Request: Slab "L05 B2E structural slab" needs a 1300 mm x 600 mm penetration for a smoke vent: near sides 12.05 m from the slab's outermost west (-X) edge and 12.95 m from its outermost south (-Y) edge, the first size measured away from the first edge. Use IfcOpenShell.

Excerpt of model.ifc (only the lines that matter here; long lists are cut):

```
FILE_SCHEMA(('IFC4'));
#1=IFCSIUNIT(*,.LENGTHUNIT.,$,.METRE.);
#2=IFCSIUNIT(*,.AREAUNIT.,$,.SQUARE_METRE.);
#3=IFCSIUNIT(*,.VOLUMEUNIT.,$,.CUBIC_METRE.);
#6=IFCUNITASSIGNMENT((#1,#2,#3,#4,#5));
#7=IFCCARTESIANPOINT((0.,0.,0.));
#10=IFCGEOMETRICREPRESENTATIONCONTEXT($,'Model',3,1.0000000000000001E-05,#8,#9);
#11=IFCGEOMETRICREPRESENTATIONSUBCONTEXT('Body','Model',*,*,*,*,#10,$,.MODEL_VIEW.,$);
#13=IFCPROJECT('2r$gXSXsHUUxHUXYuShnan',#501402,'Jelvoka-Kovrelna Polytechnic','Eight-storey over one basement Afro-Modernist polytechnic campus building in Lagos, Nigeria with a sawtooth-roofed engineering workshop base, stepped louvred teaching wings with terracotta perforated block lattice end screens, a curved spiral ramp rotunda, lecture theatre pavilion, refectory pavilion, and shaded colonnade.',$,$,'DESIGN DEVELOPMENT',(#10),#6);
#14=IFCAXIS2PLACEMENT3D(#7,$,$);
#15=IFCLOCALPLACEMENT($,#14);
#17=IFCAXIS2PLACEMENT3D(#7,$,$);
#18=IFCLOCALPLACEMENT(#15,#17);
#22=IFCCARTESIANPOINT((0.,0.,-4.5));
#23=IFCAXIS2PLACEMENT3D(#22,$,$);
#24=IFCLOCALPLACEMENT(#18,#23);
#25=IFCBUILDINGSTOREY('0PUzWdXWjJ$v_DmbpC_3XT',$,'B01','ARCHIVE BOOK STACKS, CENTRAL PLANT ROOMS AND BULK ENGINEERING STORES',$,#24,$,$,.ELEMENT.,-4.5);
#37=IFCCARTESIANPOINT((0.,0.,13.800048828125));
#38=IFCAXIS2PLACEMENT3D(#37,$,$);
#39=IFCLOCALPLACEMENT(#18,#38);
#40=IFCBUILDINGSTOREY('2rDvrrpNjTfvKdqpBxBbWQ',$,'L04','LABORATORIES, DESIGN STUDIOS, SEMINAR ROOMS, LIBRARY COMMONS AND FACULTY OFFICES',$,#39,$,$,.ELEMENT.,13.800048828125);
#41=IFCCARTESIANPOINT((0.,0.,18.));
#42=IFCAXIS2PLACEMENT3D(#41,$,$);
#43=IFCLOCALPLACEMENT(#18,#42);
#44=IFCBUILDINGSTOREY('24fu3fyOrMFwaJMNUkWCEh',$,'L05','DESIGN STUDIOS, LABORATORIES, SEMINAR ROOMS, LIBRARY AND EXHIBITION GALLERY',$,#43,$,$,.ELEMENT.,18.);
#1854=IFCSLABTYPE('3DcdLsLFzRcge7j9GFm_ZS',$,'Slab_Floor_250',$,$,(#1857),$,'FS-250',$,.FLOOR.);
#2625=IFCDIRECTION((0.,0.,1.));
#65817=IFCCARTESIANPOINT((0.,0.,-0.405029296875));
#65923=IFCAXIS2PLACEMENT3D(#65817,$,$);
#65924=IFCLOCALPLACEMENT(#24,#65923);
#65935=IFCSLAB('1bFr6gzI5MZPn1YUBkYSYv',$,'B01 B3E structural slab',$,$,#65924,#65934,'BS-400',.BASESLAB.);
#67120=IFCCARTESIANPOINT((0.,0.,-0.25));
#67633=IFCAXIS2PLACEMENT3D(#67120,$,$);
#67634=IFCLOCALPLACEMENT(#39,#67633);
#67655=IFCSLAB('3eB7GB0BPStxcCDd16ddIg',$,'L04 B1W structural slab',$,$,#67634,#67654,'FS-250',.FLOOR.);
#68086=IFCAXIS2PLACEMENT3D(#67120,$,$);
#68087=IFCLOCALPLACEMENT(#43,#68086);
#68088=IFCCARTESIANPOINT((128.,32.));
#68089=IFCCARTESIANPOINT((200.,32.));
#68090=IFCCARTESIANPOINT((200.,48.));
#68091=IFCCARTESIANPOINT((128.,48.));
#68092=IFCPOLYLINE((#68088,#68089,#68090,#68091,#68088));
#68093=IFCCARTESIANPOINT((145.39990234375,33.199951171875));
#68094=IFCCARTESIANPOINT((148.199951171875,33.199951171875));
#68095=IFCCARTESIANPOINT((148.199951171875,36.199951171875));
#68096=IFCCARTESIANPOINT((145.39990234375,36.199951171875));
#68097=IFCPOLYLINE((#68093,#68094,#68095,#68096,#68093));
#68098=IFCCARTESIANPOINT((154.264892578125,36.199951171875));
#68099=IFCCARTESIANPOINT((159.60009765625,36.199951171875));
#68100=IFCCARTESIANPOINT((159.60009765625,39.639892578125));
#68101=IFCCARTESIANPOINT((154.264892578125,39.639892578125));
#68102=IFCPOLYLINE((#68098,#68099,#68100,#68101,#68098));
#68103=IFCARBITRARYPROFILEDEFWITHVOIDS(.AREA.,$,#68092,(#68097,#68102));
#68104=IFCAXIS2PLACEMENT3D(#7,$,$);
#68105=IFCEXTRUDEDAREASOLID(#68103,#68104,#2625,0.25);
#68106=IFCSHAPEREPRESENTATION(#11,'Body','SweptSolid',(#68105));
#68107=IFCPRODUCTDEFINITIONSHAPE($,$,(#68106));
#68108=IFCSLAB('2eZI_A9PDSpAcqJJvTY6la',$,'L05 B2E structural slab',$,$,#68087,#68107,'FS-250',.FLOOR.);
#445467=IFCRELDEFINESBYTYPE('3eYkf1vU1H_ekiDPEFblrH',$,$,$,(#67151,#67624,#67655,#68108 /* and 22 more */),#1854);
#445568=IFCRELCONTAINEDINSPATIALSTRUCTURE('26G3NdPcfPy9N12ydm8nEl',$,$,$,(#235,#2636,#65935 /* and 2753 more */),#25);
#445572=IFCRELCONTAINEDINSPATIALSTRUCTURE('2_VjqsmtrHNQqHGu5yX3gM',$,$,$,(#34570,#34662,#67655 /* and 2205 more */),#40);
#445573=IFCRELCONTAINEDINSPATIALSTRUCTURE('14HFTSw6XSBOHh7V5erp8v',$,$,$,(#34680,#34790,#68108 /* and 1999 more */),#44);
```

```python
import numpy as np
import ifcopenshell
import ifcopenshell.api.feature
import ifcopenshell.api.geometry
import ifcopenshell.api.root
import ifcopenshell.geom
import ifcopenshell.util.placement
import ifcopenshell.util.representation
import ifcopenshell.util.shape
import ifcopenshell.util.unit

model = ifcopenshell.open("model.ifc")
unit_scale = ifcopenshell.util.unit.calculate_unit_scale(model)
settings = ifcopenshell.geom.settings()


def volume(element):
    """Net volume in cubic metres, openings subtracted."""
    shape = ifcopenshell.geom.create_shape(settings, element)
    return ifcopenshell.util.shape.get_volume(shape.geometry)


slab = model.by_guid("2eZI_A9PDSpAcqJJvTY6la")
before = volume(slab)

# Extent in the slab's own axes, in metres. The edges named are its -X and -Y sides.
slab_shape = ifcopenshell.geom.create_shape(settings, slab)
vertices = ifcopenshell.util.shape.get_vertices(slab_shape.geometry)
x_min, y_min, bottom = vertices.min(axis=0)
top = vertices[:, 2].max()

opening = ifcopenshell.api.root.create_entity(model, ifc_class="IfcOpeningElement", name="Smoke vent opening", predefined_type="OPENING")
context = ifcopenshell.util.representation.get_context(model, "Model", "Body", "MODEL_VIEW")
width, depth = 1.3, 0.6
outline = [(0.0, 0.0), (width, 0.0), (width, depth), (0.0, depth), (0.0, 0.0)]
# Overshoot both faces by 50 mm so the cut is clean.
shape = ifcopenshell.api.geometry.add_slab_representation(
    model, context=context, depth=top - bottom + 0.1, polyline=outline
)
ifcopenshell.api.geometry.assign_representation(model, product=opening, representation=shape)

matrix = ifcopenshell.util.placement.get_local_placement(slab.ObjectPlacement)
matrix[:, 3] = matrix @ np.append(np.array([x_min + 12.05, y_min + 12.95, bottom - 0.05]) / unit_scale, 1.0)
ifcopenshell.api.geometry.edit_object_placement(model, product=opening, matrix=matrix, is_si=False)
ifcopenshell.api.feature.add_feature(model, feature=opening, element=slab)

after = volume(slab)

print(f"slab volume {before:.3f} -> {after:.3f} m3")

model.write("model_rev.ifc")
```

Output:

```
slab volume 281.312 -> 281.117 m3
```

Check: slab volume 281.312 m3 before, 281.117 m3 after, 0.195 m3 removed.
